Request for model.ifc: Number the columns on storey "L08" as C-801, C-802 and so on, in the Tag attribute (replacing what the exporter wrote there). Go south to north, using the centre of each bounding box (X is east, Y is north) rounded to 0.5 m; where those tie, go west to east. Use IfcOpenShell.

First a look at what the model holds.

```python
import ifcopenshell
import ifcopenshell.util.element
import ifcopenshell.util.placement

model = ifcopenshell.open("model.ifc")
print(model.schema)
storey = next(s for s in model.by_type("IfcBuildingStorey") if s.Name == "L08")
columns = [e for e in ifcopenshell.util.element.get_decomposition(storey) if e.is_a("IfcColumn")]
for e in sorted(columns, key=lambda e: e.id()):
    origin = ifcopenshell.util.placement.get_local_placement(e.ObjectPlacement)[:3, 3]
    print(e.id(), e.Tag, e.Name, origin.round(2) + 0.0, sep=" | ")
```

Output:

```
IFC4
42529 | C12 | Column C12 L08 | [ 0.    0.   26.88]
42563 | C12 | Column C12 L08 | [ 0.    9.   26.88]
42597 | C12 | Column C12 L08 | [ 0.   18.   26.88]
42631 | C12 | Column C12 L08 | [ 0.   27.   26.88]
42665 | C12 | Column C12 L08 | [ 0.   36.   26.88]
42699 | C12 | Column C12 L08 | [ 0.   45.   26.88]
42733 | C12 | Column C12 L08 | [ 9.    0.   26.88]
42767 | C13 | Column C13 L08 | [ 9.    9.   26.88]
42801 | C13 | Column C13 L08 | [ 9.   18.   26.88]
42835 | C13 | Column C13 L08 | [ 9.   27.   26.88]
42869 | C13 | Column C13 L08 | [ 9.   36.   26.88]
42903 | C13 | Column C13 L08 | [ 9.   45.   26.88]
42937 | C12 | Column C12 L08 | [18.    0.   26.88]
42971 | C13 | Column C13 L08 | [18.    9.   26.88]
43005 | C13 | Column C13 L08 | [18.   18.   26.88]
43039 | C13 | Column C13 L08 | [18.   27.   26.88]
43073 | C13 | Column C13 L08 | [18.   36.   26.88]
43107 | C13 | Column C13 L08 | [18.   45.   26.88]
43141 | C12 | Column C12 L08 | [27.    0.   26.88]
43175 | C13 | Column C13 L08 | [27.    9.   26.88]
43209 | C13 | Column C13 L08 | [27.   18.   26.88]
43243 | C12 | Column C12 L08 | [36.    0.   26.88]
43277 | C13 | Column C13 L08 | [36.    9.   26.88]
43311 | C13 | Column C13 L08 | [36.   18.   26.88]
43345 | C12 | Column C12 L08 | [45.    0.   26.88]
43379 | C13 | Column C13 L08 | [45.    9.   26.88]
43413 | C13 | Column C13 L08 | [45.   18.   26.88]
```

```python
import ifcopenshell
import ifcopenshell.geom
import ifcopenshell.util.element
import ifcopenshell.util.shape

model = ifcopenshell.open("model.ifc")
settings = ifcopenshell.geom.settings()
settings.set("use-world-coords", True)


def centre(element):
    shape = ifcopenshell.geom.create_shape(settings, element)
    return ifcopenshell.util.shape.get_bbox_centroid(shape.geometry)


storey = next(s for s in model.by_type("IfcBuildingStorey") if s.Name == "L08")
columns = [e for e in ifcopenshell.util.element.get_decomposition(storey) if e.is_a("IfcColumn")]

# Insertion points can sit at a corner or the storey origin, so sort by the geometry (in metres).
centres = {e: centre(e) for e in columns}
columns.sort(key=lambda e: (round(centres[e][1] / 0.5), centres[e][0]))

for i, e in enumerate(columns, start=1):
    number = f"C-8{i:02d}"
    e.Tag = number
    print(e.id(), number)

model.write("model-out.ifc")
```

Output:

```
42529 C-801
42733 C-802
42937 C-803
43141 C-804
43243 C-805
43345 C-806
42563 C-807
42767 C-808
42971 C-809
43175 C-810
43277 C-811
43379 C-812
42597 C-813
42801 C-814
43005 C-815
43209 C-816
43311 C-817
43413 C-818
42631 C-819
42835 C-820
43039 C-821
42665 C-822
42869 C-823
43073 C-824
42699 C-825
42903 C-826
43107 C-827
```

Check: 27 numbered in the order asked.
